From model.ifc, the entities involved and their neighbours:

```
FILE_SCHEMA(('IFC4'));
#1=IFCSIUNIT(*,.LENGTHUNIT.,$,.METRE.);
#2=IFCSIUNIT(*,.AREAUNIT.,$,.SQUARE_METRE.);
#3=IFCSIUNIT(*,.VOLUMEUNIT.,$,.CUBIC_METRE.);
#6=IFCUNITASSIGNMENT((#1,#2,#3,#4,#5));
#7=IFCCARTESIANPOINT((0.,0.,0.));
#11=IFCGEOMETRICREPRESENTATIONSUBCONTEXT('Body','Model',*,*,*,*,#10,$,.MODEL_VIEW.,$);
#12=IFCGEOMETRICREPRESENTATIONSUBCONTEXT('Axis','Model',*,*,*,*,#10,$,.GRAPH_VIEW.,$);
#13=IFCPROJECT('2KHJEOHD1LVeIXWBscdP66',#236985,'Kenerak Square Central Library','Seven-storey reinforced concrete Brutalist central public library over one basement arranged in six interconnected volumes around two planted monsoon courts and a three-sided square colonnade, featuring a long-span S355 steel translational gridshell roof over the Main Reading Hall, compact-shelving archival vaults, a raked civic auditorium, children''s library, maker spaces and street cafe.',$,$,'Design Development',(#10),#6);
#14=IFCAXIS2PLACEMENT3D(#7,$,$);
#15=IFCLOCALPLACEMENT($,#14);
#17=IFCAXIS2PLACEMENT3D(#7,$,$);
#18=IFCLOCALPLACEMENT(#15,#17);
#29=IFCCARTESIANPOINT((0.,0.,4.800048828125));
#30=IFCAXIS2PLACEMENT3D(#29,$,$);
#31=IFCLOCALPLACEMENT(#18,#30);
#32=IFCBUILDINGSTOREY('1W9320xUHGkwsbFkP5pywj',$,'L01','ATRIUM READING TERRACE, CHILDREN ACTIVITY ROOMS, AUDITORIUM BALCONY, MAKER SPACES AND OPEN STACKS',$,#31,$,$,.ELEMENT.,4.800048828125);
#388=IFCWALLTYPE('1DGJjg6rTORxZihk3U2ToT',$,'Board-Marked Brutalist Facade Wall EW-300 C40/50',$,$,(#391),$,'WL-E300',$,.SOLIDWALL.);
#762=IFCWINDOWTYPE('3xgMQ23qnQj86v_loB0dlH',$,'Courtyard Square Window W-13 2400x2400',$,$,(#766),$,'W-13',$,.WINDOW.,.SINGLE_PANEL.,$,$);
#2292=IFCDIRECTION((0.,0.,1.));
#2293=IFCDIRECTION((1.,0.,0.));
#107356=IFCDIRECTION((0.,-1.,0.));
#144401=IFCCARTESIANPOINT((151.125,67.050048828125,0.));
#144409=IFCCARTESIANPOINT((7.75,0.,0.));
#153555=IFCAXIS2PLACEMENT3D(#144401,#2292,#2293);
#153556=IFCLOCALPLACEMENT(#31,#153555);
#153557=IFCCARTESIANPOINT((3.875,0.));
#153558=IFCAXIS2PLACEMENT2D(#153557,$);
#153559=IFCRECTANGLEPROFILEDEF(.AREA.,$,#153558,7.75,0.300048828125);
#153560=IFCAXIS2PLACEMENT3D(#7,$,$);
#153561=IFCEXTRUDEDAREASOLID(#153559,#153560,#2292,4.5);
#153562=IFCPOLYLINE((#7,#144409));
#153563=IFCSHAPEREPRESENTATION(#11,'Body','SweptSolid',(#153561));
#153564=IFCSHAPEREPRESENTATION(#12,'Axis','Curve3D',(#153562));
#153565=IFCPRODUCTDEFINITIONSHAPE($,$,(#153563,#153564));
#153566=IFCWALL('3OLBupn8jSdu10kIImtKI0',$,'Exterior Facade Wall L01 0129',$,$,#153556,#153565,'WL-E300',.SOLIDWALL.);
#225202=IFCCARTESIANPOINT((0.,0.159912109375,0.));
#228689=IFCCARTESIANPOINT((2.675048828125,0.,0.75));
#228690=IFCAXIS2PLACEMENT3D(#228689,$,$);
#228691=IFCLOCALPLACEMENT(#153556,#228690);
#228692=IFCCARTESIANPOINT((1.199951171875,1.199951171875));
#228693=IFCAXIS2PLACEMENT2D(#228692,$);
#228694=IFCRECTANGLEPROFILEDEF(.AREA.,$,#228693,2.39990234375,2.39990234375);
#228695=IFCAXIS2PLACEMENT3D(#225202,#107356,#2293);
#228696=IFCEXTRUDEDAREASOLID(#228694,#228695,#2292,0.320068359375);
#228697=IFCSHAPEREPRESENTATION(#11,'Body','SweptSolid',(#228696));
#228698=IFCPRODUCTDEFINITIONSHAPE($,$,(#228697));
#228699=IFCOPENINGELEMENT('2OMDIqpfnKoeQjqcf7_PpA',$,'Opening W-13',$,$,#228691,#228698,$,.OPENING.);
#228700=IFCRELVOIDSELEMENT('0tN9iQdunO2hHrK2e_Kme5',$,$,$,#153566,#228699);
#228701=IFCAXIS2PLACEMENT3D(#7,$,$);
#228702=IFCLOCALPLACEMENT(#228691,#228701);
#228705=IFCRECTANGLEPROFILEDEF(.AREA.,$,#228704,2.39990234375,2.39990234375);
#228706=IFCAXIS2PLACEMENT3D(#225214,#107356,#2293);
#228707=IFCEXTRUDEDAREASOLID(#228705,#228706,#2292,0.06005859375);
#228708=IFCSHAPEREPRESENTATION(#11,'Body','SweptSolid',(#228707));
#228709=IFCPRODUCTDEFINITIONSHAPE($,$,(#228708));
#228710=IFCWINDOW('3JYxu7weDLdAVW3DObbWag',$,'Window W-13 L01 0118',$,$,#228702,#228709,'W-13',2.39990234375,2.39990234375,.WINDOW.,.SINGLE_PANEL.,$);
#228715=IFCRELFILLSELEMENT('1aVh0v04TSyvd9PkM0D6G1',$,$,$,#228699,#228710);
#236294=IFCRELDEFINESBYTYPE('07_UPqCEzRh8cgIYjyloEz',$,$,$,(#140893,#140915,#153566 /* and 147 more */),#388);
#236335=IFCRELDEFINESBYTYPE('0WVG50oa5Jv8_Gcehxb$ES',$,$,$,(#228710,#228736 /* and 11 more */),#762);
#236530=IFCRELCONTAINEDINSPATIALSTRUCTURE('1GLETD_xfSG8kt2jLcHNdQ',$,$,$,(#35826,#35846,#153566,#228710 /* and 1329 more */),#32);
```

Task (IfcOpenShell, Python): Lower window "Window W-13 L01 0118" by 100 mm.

```python
import numpy as np
import ifcopenshell
import ifcopenshell.api.geometry
import ifcopenshell.util.placement
import ifcopenshell.util.unit

model = ifcopenshell.open("model.ifc")
unit_scale = ifcopenshell.util.unit.calculate_unit_scale(model)

window = model.by_guid("3JYxu7weDLdAVW3DObbWag")
opening = window.FillsVoids[0].RelatingOpeningElement
dz = -0.1 / unit_scale

shift = np.array([0.0, 0.0, dz])
# The window is placed relative to its opening, so it follows when the opening moves.
matrix = ifcopenshell.util.placement.get_local_placement(opening.ObjectPlacement)
matrix[:3, 3] += shift
ifcopenshell.api.geometry.edit_object_placement(
    model, product=opening, matrix=matrix, is_si=False, should_transform_children=True
)

print(f"moved by {dz * unit_scale:+.3f} m")

model.write("model_updated.ifc")
```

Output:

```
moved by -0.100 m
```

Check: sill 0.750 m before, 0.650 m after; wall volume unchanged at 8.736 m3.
